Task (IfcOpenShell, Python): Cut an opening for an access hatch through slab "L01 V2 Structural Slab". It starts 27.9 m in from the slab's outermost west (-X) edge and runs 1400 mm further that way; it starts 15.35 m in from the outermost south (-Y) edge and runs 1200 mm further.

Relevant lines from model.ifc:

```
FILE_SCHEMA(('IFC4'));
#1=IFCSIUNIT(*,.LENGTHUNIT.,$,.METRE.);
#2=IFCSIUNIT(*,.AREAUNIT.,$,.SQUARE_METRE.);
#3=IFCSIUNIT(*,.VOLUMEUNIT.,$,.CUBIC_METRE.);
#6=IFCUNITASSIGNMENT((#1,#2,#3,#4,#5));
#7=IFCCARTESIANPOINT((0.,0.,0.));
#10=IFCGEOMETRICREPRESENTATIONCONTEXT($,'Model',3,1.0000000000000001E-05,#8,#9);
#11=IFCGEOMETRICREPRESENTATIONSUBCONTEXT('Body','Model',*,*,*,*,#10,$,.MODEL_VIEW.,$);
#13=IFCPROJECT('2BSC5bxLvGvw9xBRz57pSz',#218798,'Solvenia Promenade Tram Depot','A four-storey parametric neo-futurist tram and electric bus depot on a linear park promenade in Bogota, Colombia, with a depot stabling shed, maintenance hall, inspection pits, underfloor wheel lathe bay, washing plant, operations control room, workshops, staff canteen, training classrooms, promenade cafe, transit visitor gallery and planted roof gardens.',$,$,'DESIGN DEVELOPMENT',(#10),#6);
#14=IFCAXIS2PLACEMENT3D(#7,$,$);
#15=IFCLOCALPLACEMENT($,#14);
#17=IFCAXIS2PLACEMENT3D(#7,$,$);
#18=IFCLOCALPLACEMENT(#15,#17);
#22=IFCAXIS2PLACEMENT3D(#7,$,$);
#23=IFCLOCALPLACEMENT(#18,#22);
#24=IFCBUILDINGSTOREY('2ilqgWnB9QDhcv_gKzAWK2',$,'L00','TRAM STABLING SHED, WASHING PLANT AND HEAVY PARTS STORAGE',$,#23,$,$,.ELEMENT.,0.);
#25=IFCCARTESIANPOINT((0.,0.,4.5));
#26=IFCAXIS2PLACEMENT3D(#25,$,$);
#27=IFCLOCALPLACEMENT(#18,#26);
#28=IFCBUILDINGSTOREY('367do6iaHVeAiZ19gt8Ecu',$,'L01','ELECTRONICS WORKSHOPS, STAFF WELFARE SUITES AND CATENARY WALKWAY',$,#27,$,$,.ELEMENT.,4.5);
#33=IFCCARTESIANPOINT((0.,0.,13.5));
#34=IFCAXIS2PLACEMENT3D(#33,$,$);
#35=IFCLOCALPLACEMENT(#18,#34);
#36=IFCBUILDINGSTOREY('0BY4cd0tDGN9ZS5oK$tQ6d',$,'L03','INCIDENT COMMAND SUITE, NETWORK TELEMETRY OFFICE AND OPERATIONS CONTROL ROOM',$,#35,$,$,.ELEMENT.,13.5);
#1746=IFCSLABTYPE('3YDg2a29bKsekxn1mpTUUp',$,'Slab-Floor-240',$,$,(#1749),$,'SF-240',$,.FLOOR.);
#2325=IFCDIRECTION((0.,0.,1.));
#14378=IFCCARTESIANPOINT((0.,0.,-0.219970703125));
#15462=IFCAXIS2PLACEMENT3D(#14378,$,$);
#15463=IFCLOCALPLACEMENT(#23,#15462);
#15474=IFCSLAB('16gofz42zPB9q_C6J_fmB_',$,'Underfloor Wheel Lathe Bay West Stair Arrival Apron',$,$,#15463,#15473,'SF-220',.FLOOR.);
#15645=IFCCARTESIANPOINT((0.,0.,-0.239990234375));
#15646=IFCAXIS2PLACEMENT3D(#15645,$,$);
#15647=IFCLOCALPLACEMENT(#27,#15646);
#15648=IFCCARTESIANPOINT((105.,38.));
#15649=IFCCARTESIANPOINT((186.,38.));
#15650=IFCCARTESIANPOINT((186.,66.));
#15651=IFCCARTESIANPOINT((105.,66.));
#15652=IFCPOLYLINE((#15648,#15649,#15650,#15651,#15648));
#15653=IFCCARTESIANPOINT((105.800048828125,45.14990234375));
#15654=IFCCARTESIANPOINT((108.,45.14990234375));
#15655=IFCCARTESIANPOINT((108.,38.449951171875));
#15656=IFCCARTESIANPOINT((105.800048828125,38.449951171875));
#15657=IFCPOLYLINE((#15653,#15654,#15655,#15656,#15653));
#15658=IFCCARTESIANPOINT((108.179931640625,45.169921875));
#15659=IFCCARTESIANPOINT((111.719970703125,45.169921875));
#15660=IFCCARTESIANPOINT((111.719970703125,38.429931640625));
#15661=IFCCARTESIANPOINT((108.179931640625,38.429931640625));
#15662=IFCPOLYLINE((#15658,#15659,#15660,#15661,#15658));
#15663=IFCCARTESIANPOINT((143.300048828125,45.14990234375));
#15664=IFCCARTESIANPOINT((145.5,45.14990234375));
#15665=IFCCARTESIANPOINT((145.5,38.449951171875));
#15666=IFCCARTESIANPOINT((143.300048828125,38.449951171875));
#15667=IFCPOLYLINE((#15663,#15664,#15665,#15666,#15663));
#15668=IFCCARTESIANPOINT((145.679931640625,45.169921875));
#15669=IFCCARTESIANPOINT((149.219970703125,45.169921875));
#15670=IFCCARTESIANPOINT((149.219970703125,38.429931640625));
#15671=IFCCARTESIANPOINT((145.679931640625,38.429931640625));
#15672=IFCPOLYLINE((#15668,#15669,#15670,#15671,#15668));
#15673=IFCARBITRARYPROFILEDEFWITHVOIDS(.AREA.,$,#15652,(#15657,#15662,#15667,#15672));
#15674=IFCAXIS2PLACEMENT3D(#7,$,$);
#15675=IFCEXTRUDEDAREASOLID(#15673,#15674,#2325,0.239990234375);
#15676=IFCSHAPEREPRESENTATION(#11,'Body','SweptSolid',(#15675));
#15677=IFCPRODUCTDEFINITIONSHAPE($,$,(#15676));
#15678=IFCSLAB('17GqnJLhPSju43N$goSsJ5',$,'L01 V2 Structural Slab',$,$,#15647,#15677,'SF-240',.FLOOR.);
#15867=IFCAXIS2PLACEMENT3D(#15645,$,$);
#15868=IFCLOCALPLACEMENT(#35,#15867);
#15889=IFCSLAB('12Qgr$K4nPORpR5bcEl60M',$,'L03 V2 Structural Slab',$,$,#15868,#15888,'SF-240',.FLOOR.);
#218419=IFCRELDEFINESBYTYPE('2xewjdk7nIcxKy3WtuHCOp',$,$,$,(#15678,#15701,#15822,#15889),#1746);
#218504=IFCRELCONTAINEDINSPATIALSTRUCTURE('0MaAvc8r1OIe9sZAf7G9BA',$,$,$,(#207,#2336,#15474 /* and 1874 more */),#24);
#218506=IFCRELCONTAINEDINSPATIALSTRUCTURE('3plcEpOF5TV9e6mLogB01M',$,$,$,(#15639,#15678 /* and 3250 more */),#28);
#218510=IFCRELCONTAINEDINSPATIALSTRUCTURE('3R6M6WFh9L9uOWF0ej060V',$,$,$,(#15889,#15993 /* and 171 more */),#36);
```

```python
import numpy as np
import ifcopenshell
import ifcopenshell.api.feature
import ifcopenshell.api.geometry
import ifcopenshell.api.root
import ifcopenshell.geom
import ifcopenshell.util.placement
import ifcopenshell.util.representation
import ifcopenshell.util.shape
import ifcopenshell.util.unit

model = ifcopenshell.open("model.ifc")
unit_scale = ifcopenshell.util.unit.calculate_unit_scale(model)
settings = ifcopenshell.geom.settings()


def volume(element):
    """Net volume in cubic metres, openings subtracted."""
    shape = ifcopenshell.geom.create_shape(settings, element)
    return ifcopenshell.util.shape.get_volume(shape.geometry)


slab = model.by_guid("17GqnJLhPSju43N$goSsJ5")
before = volume(slab)

# Extent in the slab's own axes, in metres. The edges named are its -X and -Y sides.
slab_shape = ifcopenshell.geom.create_shape(settings, slab)
vertices = ifcopenshell.util.shape.get_vertices(slab_shape.geometry)
x_min, y_min, bottom = vertices.min(axis=0)
top = vertices[:, 2].max()

opening = ifcopenshell.api.root.create_entity(model, ifc_class="IfcOpeningElement", name="Access hatch opening", predefined_type="OPENING")
context = ifcopenshell.util.representation.get_context(model, "Model", "Body", "MODEL_VIEW")
width, depth = 1.4, 1.2
outline = [(0.0, 0.0), (width, 0.0), (width, depth), (0.0, depth), (0.0, 0.0)]
# Overshoot both faces by 50 mm so the cut is clean.
shape = ifcopenshell.api.geometry.add_slab_representation(
    model, context=context, depth=top - bottom + 0.1, polyline=outline
)
ifcopenshell.api.geometry.assign_representation(model, product=opening, representation=shape)

matrix = ifcopenshell.util.placement.get_local_placement(slab.ObjectPlacement)
matrix[:, 3] = matrix @ np.append(np.array([x_min + 27.9, y_min + 15.35, bottom - 0.05]) / unit_scale, 1.0)
ifcopenshell.api.geometry.edit_object_placement(model, product=opening, matrix=matrix, is_si=False)
ifcopenshell.api.feature.add_feature(model, feature=opening, element=slab)

after = volume(slab)

print(f"slab volume {before:.3f} -> {after:.3f} m3")

model.write("model-out.ifc")
```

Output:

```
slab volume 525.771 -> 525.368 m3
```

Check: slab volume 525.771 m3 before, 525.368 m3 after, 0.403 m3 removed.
